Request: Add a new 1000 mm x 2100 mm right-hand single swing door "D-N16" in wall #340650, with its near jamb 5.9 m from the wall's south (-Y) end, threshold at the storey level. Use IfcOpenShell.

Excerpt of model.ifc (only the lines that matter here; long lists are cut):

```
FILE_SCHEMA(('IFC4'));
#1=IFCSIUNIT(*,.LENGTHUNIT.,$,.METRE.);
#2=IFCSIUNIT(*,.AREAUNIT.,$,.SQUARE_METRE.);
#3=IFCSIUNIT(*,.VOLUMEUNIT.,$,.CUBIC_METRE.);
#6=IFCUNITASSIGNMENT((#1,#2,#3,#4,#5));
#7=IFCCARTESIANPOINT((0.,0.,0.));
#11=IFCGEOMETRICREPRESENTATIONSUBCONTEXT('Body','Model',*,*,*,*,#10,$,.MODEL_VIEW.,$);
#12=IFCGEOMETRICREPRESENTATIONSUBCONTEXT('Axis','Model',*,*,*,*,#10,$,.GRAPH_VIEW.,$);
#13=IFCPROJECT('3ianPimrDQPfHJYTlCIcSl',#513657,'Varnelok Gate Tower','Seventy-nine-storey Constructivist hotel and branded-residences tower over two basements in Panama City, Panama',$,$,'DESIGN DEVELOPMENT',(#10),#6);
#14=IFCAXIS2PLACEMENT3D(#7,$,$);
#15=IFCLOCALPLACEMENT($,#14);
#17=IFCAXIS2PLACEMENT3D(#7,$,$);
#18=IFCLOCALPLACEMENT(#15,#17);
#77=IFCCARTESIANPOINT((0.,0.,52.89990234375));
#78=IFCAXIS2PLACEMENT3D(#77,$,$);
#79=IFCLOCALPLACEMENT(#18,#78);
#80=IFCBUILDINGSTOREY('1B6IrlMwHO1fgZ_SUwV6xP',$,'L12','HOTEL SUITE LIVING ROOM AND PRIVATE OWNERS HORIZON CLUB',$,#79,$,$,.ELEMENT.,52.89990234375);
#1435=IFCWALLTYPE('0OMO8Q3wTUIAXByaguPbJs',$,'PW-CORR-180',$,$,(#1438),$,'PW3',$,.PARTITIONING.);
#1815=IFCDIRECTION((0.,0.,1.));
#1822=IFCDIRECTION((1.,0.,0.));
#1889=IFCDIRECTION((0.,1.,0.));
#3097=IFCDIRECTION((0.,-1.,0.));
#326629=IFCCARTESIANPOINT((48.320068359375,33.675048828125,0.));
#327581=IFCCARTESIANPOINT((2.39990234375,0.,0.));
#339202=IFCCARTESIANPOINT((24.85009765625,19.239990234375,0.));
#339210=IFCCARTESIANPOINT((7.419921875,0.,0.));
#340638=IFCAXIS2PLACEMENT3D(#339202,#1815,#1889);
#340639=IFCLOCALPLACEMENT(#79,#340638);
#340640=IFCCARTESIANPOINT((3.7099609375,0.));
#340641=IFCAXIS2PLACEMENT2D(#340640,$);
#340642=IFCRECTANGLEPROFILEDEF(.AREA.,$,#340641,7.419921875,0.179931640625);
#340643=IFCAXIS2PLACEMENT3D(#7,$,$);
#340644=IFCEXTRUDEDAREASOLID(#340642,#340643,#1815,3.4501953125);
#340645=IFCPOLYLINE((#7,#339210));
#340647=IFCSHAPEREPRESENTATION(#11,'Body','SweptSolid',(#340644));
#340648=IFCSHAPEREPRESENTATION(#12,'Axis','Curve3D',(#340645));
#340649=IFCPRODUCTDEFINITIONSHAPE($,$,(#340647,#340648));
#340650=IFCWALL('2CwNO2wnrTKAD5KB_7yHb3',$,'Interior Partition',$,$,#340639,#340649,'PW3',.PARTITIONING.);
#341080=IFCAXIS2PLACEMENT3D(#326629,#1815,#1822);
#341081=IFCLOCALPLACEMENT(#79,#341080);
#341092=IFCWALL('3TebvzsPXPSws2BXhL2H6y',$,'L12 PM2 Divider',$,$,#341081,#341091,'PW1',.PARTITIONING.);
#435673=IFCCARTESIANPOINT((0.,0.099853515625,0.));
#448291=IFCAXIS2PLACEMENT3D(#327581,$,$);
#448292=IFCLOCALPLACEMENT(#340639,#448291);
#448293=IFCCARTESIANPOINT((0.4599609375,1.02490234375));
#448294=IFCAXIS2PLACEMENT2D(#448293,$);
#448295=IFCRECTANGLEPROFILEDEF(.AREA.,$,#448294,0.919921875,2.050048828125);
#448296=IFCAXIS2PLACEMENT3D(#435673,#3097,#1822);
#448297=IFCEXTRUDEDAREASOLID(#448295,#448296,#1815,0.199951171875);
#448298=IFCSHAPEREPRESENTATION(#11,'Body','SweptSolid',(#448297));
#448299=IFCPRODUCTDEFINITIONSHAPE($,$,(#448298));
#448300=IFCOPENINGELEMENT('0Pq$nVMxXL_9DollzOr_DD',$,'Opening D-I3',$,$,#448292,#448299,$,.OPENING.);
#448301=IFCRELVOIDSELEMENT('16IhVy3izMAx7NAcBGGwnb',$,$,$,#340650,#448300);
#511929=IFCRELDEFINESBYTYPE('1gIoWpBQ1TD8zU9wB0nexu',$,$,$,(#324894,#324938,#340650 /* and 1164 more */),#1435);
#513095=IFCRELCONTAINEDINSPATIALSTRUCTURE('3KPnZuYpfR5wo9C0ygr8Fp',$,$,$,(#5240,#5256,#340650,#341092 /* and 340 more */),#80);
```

```python
import numpy as np
import ifcopenshell
import ifcopenshell.api.feature
import ifcopenshell.api.geometry
import ifcopenshell.api.root
import ifcopenshell.api.spatial
import ifcopenshell.geom
import ifcopenshell.util.element
import ifcopenshell.util.placement
import ifcopenshell.util.representation
import ifcopenshell.util.shape
import ifcopenshell.util.unit

model = ifcopenshell.open("model.ifc")
unit_scale = ifcopenshell.util.unit.calculate_unit_scale(model)
settings = ifcopenshell.geom.settings()


def volume(element):
    """Net volume in cubic metres, openings subtracted."""
    shape = ifcopenshell.geom.create_shape(settings, element)
    return ifcopenshell.util.shape.get_volume(shape.geometry)


wall = model.by_id(340650)
storey = ifcopenshell.util.element.get_container(wall, ifc_class="IfcBuildingStorey")
context = ifcopenshell.util.representation.get_context(model, "Model", "Body", "MODEL_VIEW")
before = volume(wall)

width, height, from_end, sill = 1, 2.1, 5.9, 0.0  # metres

# The wall runs along its own X axis, and the end named is its -X end.
wall_shape = ifcopenshell.geom.create_shape(settings, wall)
x, y, z = ifcopenshell.util.shape.get_vertices(wall_shape.geometry).T
start = x.min() + from_end
face, thickness = float(y.min()), float(y.max() - y.min())
wall_matrix = ifcopenshell.util.placement.get_local_placement(wall.ObjectPlacement)
level = ifcopenshell.util.placement.get_local_placement(storey.ObjectPlacement)[2, 3]


def in_wall(x, y):
    """Placement at x, y metres in the wall's axes, at sill height."""
    matrix = wall_matrix.copy()
    matrix[:, 3] = wall_matrix @ np.array([x / unit_scale, y / unit_scale, 0.0, 1.0])
    matrix[2, 3] = level + sill / unit_scale
    return matrix


# Opening: a box that overshoots both wall faces by 50 mm.
opening = ifcopenshell.api.root.create_entity(model, ifc_class="IfcOpeningElement", predefined_type="OPENING")
box = ifcopenshell.api.geometry.add_wall_representation(
    model, context=context, length=width, height=height, thickness=thickness + 0.1
)
ifcopenshell.api.geometry.assign_representation(model, product=opening, representation=box)
ifcopenshell.api.geometry.edit_object_placement(model, product=opening, matrix=in_wall(start, face - 0.05), is_si=False)
ifcopenshell.api.feature.add_feature(model, feature=opening, element=wall)

door = ifcopenshell.api.root.create_entity(model, ifc_class="IfcDoor", name="D-N16", predefined_type="DOOR")
door.OverallWidth, door.OverallHeight = width / unit_scale, height / unit_scale
door.OperationType = "SINGLE_SWING_RIGHT"
body = ifcopenshell.api.geometry.add_door_representation(
    model,
    context=context,
    overall_width=door.OverallWidth,
    overall_height=door.OverallHeight,
    operation_type="SINGLE_SWING_RIGHT",
    lining_properties={"LiningDepth": thickness / unit_scale, "ThresholdDepth": thickness / unit_scale},
)
ifcopenshell.api.geometry.assign_representation(model, product=door, representation=body)
ifcopenshell.api.spatial.assign_container(model, products=[door], relating_structure=storey)
ifcopenshell.api.feature.add_filling(model, opening=opening, element=door)

# The lining spans the wall, so the door starts at the wall face.
ifcopenshell.api.geometry.edit_object_placement(model, product=door, matrix=in_wall(start, face), is_si=False)

after = volume(wall)

print(f"wall volume {before:.3f} -> {after:.3f} m3")

model.write("model_updated.ifc")
```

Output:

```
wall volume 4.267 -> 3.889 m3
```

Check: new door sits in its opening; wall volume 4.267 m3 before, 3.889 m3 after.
